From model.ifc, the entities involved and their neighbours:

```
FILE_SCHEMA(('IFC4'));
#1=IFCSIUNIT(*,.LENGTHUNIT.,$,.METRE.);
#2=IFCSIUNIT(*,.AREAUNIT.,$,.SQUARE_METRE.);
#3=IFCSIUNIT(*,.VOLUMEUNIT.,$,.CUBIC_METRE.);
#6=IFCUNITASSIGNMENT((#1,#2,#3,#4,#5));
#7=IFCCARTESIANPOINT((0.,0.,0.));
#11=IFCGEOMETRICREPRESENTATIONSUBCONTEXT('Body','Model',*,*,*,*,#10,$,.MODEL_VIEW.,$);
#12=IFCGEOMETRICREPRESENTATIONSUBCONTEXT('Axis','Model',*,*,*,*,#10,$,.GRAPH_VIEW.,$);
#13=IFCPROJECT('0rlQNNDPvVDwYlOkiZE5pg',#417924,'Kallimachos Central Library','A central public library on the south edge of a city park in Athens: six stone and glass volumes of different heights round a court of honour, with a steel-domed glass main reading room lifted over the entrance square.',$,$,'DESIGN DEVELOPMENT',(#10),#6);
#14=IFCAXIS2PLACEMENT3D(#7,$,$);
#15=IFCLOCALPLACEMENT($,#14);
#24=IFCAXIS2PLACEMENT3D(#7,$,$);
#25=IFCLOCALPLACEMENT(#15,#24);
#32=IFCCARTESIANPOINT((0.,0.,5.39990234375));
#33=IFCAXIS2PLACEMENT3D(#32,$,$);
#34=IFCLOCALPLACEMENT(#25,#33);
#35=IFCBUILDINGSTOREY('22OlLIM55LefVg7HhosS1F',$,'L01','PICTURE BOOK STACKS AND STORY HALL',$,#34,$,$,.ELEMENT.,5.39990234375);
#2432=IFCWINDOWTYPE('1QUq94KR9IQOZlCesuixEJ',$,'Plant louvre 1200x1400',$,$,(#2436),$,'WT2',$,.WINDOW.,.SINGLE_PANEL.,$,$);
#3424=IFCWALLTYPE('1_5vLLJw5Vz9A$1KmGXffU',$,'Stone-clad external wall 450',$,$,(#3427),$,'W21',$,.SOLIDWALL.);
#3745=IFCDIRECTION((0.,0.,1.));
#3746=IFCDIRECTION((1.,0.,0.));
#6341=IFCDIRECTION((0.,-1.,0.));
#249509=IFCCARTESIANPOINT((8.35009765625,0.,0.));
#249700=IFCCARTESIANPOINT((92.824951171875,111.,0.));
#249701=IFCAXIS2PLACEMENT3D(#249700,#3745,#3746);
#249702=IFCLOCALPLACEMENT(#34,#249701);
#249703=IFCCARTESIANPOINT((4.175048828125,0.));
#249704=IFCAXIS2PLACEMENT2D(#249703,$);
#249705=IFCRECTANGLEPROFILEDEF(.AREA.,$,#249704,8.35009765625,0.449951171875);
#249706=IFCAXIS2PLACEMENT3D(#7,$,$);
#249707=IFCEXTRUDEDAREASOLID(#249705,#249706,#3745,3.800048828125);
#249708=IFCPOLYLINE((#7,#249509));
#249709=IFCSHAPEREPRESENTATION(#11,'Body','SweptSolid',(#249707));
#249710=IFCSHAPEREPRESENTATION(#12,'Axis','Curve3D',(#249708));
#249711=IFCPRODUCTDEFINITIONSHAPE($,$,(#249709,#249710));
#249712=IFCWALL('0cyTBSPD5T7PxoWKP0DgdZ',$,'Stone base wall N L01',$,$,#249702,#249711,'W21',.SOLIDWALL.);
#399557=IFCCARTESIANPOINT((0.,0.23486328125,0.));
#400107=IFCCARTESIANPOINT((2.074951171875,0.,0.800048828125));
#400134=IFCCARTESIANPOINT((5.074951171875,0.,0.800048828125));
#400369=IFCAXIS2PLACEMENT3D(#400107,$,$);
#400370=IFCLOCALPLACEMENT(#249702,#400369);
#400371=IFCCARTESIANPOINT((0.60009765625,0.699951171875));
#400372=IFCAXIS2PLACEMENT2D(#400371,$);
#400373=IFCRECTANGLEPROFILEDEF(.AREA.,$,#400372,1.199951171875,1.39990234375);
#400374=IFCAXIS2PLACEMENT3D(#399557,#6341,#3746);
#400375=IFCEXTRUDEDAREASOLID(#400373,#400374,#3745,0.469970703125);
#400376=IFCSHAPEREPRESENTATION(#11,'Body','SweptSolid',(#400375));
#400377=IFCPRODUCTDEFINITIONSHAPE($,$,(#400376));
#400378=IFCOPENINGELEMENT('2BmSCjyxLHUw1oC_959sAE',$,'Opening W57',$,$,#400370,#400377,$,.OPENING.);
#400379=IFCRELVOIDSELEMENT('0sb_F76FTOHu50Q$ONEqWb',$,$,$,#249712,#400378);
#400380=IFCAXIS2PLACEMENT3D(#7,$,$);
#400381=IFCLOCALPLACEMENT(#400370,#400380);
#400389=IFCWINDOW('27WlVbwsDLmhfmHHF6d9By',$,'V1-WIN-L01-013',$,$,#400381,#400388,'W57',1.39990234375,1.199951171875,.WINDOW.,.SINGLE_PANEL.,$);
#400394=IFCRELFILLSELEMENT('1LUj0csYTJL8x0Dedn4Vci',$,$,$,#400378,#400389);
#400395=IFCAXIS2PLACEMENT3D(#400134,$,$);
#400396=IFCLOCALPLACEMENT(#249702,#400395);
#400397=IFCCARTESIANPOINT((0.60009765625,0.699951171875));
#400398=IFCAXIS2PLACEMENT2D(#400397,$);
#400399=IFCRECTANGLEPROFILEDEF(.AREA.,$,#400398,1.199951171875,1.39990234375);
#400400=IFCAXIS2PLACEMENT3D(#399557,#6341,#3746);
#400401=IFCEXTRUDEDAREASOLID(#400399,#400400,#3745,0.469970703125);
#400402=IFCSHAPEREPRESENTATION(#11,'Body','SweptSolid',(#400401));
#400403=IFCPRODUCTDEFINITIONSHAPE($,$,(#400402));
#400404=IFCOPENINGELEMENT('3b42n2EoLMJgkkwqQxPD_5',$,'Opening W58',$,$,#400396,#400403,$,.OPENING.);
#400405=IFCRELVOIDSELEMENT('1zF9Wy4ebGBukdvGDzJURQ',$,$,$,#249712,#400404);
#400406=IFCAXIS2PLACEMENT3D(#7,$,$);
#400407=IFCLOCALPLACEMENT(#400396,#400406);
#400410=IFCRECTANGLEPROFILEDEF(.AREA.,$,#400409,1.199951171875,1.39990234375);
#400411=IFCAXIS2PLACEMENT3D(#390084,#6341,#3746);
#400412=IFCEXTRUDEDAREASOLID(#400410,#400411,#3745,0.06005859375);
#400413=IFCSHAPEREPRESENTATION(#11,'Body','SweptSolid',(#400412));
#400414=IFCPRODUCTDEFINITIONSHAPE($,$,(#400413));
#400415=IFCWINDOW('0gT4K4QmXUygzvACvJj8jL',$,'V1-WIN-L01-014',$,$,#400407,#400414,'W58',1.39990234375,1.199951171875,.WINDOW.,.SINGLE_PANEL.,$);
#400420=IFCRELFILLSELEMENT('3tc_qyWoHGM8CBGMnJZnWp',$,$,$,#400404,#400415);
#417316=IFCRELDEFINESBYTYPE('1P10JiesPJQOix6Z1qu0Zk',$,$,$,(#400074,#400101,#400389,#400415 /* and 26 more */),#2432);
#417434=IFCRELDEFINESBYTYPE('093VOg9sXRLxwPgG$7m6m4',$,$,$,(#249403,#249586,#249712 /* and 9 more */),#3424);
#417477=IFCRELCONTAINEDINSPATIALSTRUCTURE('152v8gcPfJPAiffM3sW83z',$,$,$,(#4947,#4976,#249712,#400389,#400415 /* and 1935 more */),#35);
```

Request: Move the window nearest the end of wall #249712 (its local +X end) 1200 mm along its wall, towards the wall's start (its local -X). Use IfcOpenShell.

```python
import ifcopenshell
import ifcopenshell.api.geometry
import ifcopenshell.util.placement
import ifcopenshell.util.unit

model = ifcopenshell.open("model.ifc")
unit_scale = ifcopenshell.util.unit.calculate_unit_scale(model)

window = model.by_guid("0gT4K4QmXUygzvACvJj8jL")
opening = window.FillsVoids[0].RelatingOpeningElement
wall = opening.VoidsElements[0].RelatingBuildingElement

wall_matrix = ifcopenshell.util.placement.get_local_placement(wall.ObjectPlacement)
shift = wall_matrix[:3, 0] * -1.2 / unit_scale
before = ifcopenshell.util.placement.get_local_placement(window.ObjectPlacement)[:3, 3].copy()

# The window is placed relative to its opening, so it follows when the opening moves.
matrix = ifcopenshell.util.placement.get_local_placement(opening.ObjectPlacement)
matrix[:3, 3] += shift
ifcopenshell.api.geometry.edit_object_placement(
    model, product=opening, matrix=matrix, is_si=False, should_transform_children=True
)

after = ifcopenshell.util.placement.get_local_placement(window.ObjectPlacement)[:3, 3]
print("window moved by", (after - before).round(3) + 0.0)

model.write("model_rev.ifc")
```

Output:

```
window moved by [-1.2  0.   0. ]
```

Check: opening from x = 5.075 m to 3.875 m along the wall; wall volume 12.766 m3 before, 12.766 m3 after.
